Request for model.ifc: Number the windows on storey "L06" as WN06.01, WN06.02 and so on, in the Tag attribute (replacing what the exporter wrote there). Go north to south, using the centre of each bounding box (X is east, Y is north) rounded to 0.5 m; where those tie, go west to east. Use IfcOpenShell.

First a look at what the model holds.

```python
import ifcopenshell
import ifcopenshell.util.element
import ifcopenshell.util.placement

model = ifcopenshell.open("model.ifc")
print(model.schema)
storey = next(s for s in model.by_type("IfcBuildingStorey") if s.Name == "L06")
windows = [e for e in ifcopenshell.util.element.get_decomposition(storey) if e.is_a("IfcWindow")]
for e in sorted(windows, key=lambda e: e.id()):
    origin = ifcopenshell.util.placement.get_local_placement(e.ObjectPlacement)[:3, 3]
    print(e.id(), e.Tag, e.Name, origin.round(2) + 0.0, sep=" | ")
```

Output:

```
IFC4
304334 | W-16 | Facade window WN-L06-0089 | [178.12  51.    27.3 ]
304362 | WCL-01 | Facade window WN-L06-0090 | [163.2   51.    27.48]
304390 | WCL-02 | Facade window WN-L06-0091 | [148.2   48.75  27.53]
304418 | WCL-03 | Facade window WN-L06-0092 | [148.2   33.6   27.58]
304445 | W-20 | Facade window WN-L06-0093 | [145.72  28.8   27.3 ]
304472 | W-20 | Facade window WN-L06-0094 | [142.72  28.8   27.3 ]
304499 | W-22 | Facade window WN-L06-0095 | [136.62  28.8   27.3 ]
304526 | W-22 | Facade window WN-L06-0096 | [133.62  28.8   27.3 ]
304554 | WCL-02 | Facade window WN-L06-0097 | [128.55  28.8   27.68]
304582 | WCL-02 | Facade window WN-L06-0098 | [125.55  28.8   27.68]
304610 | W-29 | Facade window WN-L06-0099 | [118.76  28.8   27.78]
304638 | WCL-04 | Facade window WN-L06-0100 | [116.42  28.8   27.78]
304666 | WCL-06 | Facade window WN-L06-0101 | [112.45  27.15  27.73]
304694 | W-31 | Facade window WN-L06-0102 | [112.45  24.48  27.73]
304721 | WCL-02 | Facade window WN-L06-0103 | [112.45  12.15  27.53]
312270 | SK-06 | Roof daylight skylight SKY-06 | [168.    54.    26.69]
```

```python
import ifcopenshell
import ifcopenshell.geom
import ifcopenshell.util.element
import ifcopenshell.util.shape

model = ifcopenshell.open("model.ifc")
settings = ifcopenshell.geom.settings()
settings.set("use-world-coords", True)


def centre(element):
    shape = ifcopenshell.geom.create_shape(settings, element)
    return ifcopenshell.util.shape.get_bbox_centroid(shape.geometry)


storey = next(s for s in model.by_type("IfcBuildingStorey") if s.Name == "L06")
windows = [e for e in ifcopenshell.util.element.get_decomposition(storey) if e.is_a("IfcWindow")]

# Insertion points can sit at a corner or the storey origin, so sort by the geometry (in metres).
centres = {e: centre(e) for e in windows}
windows.sort(key=lambda e: (-round(centres[e][1] / 0.5), centres[e][0]))

for i, e in enumerate(windows, start=1):
    number = f"WN06.{i:02d}"
    e.Tag = number
    print(e.id(), number)

model.write("model-out.ifc")
```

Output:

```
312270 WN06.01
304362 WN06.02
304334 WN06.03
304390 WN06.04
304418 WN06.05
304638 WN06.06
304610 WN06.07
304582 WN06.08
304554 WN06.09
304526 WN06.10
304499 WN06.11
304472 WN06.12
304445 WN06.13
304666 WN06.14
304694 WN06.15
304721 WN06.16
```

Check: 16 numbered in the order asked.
